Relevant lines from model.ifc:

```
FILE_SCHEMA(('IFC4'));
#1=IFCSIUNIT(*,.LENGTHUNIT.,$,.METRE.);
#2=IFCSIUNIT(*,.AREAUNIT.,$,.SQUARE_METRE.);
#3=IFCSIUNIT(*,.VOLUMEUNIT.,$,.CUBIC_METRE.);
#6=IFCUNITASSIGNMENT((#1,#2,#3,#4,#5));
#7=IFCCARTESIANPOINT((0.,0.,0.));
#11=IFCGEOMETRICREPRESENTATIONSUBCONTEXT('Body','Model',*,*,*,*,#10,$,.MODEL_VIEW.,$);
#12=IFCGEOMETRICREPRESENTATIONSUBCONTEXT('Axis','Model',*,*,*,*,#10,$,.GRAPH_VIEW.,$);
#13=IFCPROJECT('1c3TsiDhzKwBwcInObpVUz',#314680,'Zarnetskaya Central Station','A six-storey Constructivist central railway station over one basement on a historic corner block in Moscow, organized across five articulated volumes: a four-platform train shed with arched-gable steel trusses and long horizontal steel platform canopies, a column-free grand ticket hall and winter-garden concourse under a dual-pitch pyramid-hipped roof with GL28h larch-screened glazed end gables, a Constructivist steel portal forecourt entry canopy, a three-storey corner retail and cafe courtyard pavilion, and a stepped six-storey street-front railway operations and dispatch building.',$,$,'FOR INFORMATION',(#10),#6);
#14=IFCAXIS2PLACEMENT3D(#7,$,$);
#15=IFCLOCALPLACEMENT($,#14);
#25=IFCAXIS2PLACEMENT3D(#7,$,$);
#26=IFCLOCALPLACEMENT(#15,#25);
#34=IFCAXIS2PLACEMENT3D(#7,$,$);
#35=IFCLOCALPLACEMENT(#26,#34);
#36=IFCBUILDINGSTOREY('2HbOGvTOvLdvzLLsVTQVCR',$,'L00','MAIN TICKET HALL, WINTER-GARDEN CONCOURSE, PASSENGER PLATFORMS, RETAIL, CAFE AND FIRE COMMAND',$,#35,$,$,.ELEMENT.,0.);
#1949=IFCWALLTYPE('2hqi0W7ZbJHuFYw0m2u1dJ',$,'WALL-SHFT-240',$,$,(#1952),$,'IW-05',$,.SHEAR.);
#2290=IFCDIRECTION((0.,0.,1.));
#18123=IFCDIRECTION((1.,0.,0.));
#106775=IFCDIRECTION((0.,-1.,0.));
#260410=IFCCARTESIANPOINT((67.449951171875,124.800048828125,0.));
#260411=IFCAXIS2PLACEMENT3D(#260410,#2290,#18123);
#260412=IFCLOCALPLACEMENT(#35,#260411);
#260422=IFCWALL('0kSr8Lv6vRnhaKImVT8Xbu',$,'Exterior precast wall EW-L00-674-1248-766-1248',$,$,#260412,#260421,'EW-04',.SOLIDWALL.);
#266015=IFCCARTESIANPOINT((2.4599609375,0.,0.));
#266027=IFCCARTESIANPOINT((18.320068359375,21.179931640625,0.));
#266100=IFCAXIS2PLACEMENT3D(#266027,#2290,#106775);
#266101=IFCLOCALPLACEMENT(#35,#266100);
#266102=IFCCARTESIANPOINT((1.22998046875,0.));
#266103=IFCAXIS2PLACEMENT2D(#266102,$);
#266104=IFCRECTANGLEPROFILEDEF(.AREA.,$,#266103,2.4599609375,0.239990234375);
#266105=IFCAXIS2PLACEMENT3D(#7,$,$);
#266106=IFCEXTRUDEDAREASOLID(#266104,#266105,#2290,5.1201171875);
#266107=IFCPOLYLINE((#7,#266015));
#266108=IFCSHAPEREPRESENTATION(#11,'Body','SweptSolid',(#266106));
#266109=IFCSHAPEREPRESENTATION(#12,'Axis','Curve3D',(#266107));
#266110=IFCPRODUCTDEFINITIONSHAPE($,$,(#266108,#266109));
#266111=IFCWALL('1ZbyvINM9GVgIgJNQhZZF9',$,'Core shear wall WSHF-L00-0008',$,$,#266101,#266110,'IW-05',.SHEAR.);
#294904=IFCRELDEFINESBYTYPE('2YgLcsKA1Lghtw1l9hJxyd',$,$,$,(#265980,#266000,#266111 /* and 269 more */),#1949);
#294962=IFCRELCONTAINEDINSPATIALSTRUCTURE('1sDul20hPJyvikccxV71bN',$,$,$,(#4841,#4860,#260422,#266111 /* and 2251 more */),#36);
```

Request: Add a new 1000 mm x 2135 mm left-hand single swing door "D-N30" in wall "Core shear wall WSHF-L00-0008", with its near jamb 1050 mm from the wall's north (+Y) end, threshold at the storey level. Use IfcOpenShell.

```python
import numpy as np
import ifcopenshell
import ifcopenshell.api.feature
import ifcopenshell.api.geometry
import ifcopenshell.api.root
import ifcopenshell.api.spatial
import ifcopenshell.geom
import ifcopenshell.util.element
import ifcopenshell.util.placement
import ifcopenshell.util.representation
import ifcopenshell.util.shape
import ifcopenshell.util.unit

model = ifcopenshell.open("model.ifc")
unit_scale = ifcopenshell.util.unit.calculate_unit_scale(model)
settings = ifcopenshell.geom.settings()


def volume(element):
    """Net volume in cubic metres, openings subtracted."""
    shape = ifcopenshell.geom.create_shape(settings, element)
    return ifcopenshell.util.shape.get_volume(shape.geometry)


wall = model.by_guid("1ZbyvINM9GVgIgJNQhZZF9")
storey = ifcopenshell.util.element.get_container(wall, ifc_class="IfcBuildingStorey")
context = ifcopenshell.util.representation.get_context(model, "Model", "Body", "MODEL_VIEW")
before = volume(wall)

width, height, from_end, sill = 1, 2.135, 1.05, 0.0  # metres

# The wall runs along its own X axis, and the end named is its -X end.
wall_shape = ifcopenshell.geom.create_shape(settings, wall)
x, y, z = ifcopenshell.util.shape.get_vertices(wall_shape.geometry).T
start = x.min() + from_end
face, thickness = float(y.min()), float(y.max() - y.min())
wall_matrix = ifcopenshell.util.placement.get_local_placement(wall.ObjectPlacement)
level = ifcopenshell.util.placement.get_local_placement(storey.ObjectPlacement)[2, 3]


def in_wall(x, y):
    """Placement at x, y metres in the wall's axes, at sill height."""
    matrix = wall_matrix.copy()
    matrix[:, 3] = wall_matrix @ np.array([x / unit_scale, y / unit_scale, 0.0, 1.0])
    matrix[2, 3] = level + sill / unit_scale
    return matrix


# Opening: a box that overshoots both wall faces by 50 mm.
opening = ifcopenshell.api.root.create_entity(model, ifc_class="IfcOpeningElement", predefined_type="OPENING")
box = ifcopenshell.api.geometry.add_wall_representation(
    model, context=context, length=width, height=height, thickness=thickness + 0.1
)
ifcopenshell.api.geometry.assign_representation(model, product=opening, representation=box)
ifcopenshell.api.geometry.edit_object_placement(model, product=opening, matrix=in_wall(start, face - 0.05), is_si=False)
ifcopenshell.api.feature.add_feature(model, feature=opening, element=wall)

door = ifcopenshell.api.root.create_entity(model, ifc_class="IfcDoor", name="D-N30", predefined_type="DOOR")
door.OverallWidth, door.OverallHeight = width / unit_scale, height / unit_scale
door.OperationType = "SINGLE_SWING_LEFT"
body = ifcopenshell.api.geometry.add_door_representation(
    model,
    context=context,
    overall_width=door.OverallWidth,
    overall_height=door.OverallHeight,
    operation_type="SINGLE_SWING_LEFT",
    lining_properties={"LiningDepth": thickness / unit_scale, "ThresholdDepth": thickness / unit_scale},
)
ifcopenshell.api.geometry.assign_representation(model, product=door, representation=body)
ifcopenshell.api.spatial.assign_container(model, products=[door], relating_structure=storey)
ifcopenshell.api.feature.add_filling(model, opening=opening, element=door)

# The lining spans the wall, so the door starts at the wall face.
ifcopenshell.api.geometry.edit_object_placement(model, product=door, matrix=in_wall(start, face), is_si=False)

after = volume(wall)

print(f"wall volume {before:.3f} -> {after:.3f} m3")

model.write("model_updated.ifc")
```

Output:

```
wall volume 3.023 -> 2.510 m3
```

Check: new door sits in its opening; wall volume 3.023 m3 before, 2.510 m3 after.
